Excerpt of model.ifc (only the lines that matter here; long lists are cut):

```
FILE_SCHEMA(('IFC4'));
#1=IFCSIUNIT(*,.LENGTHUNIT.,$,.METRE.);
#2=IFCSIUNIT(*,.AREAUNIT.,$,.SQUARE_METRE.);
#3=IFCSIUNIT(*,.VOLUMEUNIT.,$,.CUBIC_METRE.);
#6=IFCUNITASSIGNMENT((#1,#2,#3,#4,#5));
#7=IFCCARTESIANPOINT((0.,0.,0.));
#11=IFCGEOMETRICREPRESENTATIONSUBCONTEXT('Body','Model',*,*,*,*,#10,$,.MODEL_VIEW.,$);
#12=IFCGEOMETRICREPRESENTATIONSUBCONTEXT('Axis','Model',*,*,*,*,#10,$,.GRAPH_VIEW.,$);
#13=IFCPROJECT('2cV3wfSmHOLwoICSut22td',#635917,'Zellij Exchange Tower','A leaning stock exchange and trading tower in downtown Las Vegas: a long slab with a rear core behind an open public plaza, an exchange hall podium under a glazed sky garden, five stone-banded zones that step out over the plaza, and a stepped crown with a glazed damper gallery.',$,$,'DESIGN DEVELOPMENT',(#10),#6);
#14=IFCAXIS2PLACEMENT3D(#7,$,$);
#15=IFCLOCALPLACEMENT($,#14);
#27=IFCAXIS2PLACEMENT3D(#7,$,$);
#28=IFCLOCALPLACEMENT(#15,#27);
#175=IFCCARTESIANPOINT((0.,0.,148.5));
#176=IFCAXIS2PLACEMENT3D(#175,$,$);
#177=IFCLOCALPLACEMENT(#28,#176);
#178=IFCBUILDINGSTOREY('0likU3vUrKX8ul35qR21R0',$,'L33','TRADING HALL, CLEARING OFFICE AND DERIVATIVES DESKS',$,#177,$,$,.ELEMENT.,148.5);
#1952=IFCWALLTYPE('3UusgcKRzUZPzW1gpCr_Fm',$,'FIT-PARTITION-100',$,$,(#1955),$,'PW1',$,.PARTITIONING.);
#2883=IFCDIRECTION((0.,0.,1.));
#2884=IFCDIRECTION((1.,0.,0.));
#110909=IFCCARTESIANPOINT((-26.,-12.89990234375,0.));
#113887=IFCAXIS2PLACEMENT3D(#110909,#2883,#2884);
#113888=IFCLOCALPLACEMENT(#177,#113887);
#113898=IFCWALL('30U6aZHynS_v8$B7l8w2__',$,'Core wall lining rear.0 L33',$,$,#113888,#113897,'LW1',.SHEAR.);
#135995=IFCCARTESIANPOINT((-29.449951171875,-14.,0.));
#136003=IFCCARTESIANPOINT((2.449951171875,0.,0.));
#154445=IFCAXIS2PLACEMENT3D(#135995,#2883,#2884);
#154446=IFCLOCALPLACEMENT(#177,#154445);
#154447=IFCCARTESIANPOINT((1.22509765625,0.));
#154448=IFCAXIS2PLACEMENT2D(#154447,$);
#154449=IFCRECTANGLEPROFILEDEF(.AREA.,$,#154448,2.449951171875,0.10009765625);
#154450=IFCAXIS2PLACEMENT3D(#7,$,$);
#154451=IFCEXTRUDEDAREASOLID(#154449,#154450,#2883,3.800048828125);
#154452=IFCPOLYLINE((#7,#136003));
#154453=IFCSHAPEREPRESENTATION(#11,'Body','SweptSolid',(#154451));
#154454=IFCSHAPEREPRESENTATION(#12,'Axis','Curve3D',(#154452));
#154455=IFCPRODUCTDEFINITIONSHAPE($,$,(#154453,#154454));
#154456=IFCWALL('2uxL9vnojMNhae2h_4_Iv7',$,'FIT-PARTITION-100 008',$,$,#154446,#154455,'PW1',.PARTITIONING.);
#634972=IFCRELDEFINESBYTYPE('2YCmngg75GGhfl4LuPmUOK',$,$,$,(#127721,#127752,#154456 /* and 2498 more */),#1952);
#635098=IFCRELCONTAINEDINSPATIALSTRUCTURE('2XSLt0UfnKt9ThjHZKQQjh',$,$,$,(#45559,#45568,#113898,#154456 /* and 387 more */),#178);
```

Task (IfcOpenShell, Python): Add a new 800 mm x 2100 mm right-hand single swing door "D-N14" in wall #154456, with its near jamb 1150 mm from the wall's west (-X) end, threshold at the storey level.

```python
import numpy as np
import ifcopenshell
import ifcopenshell.api.feature
import ifcopenshell.api.geometry
import ifcopenshell.api.root
import ifcopenshell.api.spatial
import ifcopenshell.geom
import ifcopenshell.util.element
import ifcopenshell.util.placement
import ifcopenshell.util.representation
import ifcopenshell.util.shape
import ifcopenshell.util.unit

model = ifcopenshell.open("model.ifc")
unit_scale = ifcopenshell.util.unit.calculate_unit_scale(model)
settings = ifcopenshell.geom.settings()


def volume(element):
    """Net volume in cubic metres, openings subtracted."""
    shape = ifcopenshell.geom.create_shape(settings, element)
    return ifcopenshell.util.shape.get_volume(shape.geometry)


wall = model.by_guid("2uxL9vnojMNhae2h_4_Iv7")
storey = ifcopenshell.util.element.get_container(wall, ifc_class="IfcBuildingStorey")
context = ifcopenshell.util.representation.get_context(model, "Model", "Body", "MODEL_VIEW")
before = volume(wall)

width, height, from_end, sill = 0.8, 2.1, 1.15, 0.0  # metres

# The wall runs along its own X axis, and the end named is its -X end.
wall_shape = ifcopenshell.geom.create_shape(settings, wall)
x, y, z = ifcopenshell.util.shape.get_vertices(wall_shape.geometry).T
start = x.min() + from_end
face, thickness = float(y.min()), float(y.max() - y.min())
wall_matrix = ifcopenshell.util.placement.get_local_placement(wall.ObjectPlacement)
level = ifcopenshell.util.placement.get_local_placement(storey.ObjectPlacement)[2, 3]


def in_wall(x, y):
    """Placement at x, y metres in the wall's axes, at sill height."""
    matrix = wall_matrix.copy()
    matrix[:, 3] = wall_matrix @ np.array([x / unit_scale, y / unit_scale, 0.0, 1.0])
    matrix[2, 3] = level + sill / unit_scale
    return matrix


# Opening: a box that overshoots both wall faces by 50 mm.
opening = ifcopenshell.api.root.create_entity(model, ifc_class="IfcOpeningElement", predefined_type="OPENING")
box = ifcopenshell.api.geometry.add_wall_representation(
    model, context=context, length=width, height=height, thickness=thickness + 0.1
)
ifcopenshell.api.geometry.assign_representation(model, product=opening, representation=box)
ifcopenshell.api.geometry.edit_object_placement(model, product=opening, matrix=in_wall(start, face - 0.05), is_si=False)
ifcopenshell.api.feature.add_feature(model, feature=opening, element=wall)

door = ifcopenshell.api.root.create_entity(model, ifc_class="IfcDoor", name="D-N14", predefined_type="DOOR")
door.OverallWidth, door.OverallHeight = width / unit_scale, height / unit_scale
door.OperationType = "SINGLE_SWING_RIGHT"
body = ifcopenshell.api.geometry.add_door_representation(
    model,
    context=context,
    overall_width=door.OverallWidth,
    overall_height=door.OverallHeight,
    operation_type="SINGLE_SWING_RIGHT",
    lining_properties={"LiningDepth": thickness / unit_scale, "ThresholdDepth": thickness / unit_scale},
)
ifcopenshell.api.geometry.assign_representation(model, product=door, representation=body)
ifcopenshell.api.spatial.assign_container(model, products=[door], relating_structure=storey)
ifcopenshell.api.feature.add_filling(model, opening=opening, element=door)

# The lining spans the wall, so the door starts at the wall face.
ifcopenshell.api.geometry.edit_object_placement(model, product=door, matrix=in_wall(start, face), is_si=False)

after = volume(wall)

print(f"wall volume {before:.3f} -> {after:.3f} m3")

model.write("model_rev.ifc")
```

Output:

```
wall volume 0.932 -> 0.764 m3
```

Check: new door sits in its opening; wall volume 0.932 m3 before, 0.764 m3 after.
